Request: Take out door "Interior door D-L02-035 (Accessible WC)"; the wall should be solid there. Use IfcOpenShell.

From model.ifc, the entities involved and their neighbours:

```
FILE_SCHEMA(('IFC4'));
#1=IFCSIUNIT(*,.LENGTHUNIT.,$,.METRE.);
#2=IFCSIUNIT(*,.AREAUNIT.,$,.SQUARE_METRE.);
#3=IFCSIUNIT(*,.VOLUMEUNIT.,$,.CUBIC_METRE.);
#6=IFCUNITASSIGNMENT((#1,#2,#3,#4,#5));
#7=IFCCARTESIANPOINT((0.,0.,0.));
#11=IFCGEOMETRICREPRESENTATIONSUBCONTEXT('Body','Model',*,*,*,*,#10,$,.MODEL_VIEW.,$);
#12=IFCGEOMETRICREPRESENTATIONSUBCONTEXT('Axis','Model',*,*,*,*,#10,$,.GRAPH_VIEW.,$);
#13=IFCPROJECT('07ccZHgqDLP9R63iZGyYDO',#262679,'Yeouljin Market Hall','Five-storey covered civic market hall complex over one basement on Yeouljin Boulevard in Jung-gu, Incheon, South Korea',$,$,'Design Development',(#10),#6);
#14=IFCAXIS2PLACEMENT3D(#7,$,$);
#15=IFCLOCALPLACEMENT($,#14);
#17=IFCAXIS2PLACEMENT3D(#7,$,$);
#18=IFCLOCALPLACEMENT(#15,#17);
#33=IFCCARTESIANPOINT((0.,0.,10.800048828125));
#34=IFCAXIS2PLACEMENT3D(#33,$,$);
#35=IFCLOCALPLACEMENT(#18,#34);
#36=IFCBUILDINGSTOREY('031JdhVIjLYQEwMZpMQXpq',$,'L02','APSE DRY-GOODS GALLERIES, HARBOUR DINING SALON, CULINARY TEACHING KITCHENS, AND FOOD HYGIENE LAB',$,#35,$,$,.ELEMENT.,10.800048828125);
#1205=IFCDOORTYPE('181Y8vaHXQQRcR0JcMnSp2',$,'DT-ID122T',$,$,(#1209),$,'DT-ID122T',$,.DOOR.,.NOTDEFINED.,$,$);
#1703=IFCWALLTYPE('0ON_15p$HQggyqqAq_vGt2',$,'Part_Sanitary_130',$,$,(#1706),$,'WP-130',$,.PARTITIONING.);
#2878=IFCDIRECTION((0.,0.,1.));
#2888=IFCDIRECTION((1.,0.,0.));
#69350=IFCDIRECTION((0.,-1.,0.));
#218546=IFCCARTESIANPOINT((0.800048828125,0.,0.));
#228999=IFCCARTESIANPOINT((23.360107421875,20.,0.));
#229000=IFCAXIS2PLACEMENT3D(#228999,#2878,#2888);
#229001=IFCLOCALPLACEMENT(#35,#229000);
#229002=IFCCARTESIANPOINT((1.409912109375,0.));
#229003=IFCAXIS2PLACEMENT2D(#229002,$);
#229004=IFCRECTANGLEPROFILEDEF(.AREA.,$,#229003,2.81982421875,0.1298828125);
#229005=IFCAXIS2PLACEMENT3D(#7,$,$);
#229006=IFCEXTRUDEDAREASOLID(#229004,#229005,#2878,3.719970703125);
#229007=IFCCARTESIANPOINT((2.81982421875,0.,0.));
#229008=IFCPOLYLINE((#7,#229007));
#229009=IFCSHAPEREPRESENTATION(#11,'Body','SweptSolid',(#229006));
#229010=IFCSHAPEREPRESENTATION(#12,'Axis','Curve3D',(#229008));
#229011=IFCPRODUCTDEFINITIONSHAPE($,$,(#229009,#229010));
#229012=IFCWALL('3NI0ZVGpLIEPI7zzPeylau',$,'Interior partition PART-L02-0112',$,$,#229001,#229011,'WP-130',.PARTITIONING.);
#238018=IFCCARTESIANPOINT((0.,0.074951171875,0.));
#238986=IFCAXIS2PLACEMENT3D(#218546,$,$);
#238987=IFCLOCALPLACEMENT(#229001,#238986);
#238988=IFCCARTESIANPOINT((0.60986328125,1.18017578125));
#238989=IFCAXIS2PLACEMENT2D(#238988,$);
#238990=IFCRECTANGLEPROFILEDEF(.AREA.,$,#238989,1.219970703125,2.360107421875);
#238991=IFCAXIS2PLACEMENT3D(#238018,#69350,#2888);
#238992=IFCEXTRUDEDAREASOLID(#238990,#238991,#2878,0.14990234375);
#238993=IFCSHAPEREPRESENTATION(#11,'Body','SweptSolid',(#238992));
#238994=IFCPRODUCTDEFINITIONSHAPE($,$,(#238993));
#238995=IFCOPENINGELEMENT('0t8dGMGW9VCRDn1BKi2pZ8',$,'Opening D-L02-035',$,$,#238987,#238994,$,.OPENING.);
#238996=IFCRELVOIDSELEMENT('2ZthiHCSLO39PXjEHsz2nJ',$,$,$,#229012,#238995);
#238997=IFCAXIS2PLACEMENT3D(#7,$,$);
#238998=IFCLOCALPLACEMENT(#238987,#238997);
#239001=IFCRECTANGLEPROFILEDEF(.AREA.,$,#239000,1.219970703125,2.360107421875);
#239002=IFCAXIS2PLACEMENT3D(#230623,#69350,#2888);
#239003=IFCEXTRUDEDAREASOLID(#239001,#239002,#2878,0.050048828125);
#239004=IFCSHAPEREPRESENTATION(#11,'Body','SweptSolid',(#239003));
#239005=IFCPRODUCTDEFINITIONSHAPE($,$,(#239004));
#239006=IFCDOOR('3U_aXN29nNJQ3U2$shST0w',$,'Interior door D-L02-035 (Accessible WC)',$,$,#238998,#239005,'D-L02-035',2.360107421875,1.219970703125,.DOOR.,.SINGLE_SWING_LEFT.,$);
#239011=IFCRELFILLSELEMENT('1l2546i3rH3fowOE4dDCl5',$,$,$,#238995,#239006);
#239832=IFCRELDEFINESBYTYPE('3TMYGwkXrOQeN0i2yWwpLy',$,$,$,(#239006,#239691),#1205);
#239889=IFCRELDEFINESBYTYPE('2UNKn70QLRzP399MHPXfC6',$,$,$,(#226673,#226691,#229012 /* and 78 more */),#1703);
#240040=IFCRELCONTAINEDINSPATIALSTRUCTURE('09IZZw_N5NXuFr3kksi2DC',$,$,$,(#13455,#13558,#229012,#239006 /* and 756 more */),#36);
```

```python
import ifcopenshell
import ifcopenshell.api.feature
import ifcopenshell.api.root
import ifcopenshell.geom
import ifcopenshell.util.shape

model = ifcopenshell.open("model.ifc")
settings = ifcopenshell.geom.settings()


def volume(element):
    """Net volume in cubic metres, openings subtracted."""
    shape = ifcopenshell.geom.create_shape(settings, element)
    return ifcopenshell.util.shape.get_volume(shape.geometry)


door = model.by_guid("3U_aXN29nNJQ3U2$shST0w")
opening = door.FillsVoids[0].RelatingOpeningElement
wall = opening.VoidsElements[0].RelatingBuildingElement
before = volume(wall)

ifcopenshell.api.root.remove_product(model, product=door)
ifcopenshell.api.feature.remove_feature(model, feature=opening)

after = volume(wall)

print(f"wall volume {before:.3f} -> {after:.3f} m3")

model.write("model_rev.ifc")
```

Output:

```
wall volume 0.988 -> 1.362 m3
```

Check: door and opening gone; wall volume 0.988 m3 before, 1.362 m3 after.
